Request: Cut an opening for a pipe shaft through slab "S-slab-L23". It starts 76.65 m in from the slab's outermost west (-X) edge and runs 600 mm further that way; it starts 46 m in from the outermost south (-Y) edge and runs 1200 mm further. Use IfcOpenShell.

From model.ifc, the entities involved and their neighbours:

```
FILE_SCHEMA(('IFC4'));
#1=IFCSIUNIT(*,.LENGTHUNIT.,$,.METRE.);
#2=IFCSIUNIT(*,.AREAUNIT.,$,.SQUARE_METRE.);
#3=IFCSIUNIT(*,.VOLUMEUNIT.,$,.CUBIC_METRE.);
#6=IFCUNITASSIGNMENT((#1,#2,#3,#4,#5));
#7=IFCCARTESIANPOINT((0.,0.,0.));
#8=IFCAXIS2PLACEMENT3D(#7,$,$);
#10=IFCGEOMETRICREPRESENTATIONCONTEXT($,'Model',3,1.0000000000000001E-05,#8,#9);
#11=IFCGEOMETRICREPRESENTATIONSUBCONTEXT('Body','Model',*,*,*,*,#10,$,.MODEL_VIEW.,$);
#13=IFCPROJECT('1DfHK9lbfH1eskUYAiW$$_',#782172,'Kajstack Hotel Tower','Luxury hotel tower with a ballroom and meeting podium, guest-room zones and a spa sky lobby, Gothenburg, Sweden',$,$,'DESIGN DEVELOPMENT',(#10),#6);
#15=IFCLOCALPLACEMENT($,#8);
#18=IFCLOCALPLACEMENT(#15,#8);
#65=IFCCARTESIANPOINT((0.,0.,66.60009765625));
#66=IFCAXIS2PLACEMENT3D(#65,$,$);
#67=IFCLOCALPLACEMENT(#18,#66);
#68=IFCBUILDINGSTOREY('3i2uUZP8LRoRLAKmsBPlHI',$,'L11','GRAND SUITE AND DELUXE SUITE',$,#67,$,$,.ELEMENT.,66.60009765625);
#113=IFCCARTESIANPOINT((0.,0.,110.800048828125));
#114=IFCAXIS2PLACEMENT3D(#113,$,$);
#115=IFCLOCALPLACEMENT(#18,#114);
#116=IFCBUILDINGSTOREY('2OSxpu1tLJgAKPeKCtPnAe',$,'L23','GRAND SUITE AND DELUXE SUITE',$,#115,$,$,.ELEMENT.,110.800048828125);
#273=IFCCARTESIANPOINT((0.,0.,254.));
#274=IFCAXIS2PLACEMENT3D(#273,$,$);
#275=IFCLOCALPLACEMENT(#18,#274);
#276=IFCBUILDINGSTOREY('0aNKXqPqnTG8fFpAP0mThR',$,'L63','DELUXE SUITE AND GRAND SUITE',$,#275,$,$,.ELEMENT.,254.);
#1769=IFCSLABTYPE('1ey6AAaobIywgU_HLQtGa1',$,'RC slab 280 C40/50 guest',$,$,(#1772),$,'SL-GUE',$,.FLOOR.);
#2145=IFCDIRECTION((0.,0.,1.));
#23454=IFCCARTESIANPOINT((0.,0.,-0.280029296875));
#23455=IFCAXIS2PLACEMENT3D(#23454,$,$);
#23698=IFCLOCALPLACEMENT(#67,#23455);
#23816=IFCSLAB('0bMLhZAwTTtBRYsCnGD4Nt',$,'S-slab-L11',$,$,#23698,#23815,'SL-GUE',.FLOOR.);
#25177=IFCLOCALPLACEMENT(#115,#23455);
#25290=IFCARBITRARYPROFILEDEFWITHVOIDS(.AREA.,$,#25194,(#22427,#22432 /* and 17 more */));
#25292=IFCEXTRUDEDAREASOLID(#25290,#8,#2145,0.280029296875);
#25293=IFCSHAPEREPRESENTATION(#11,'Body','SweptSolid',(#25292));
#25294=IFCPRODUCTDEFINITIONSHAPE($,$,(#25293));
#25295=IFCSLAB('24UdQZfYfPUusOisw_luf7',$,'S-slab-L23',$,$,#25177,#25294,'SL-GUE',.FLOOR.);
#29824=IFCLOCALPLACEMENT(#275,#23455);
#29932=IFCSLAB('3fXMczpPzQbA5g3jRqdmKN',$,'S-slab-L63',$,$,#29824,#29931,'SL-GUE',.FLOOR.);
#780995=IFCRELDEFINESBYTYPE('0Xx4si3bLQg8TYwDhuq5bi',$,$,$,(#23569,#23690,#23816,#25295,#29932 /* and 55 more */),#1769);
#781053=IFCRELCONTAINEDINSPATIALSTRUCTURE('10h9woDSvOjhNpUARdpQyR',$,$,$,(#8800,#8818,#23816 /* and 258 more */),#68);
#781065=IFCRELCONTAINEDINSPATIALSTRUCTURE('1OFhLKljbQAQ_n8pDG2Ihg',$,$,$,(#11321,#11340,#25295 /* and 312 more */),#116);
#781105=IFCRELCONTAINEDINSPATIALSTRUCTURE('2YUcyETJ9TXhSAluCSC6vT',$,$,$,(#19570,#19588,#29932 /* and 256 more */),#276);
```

```python
import numpy as np
import ifcopenshell
import ifcopenshell.api.feature
import ifcopenshell.api.geometry
import ifcopenshell.api.root
import ifcopenshell.geom
import ifcopenshell.util.placement
import ifcopenshell.util.representation
import ifcopenshell.util.shape
import ifcopenshell.util.unit

model = ifcopenshell.open("model.ifc")
unit_scale = ifcopenshell.util.unit.calculate_unit_scale(model)
settings = ifcopenshell.geom.settings()


def volume(element):
    """Net volume in cubic metres, openings subtracted."""
    shape = ifcopenshell.geom.create_shape(settings, element)
    return ifcopenshell.util.shape.get_volume(shape.geometry)


slab = model.by_id(25295)
before = volume(slab)

# Extent in the slab's own axes, in metres. The edges named are its -X and -Y sides.
slab_shape = ifcopenshell.geom.create_shape(settings, slab)
vertices = ifcopenshell.util.shape.get_vertices(slab_shape.geometry)
x_min, y_min, bottom = vertices.min(axis=0)
top = vertices[:, 2].max()

opening = ifcopenshell.api.root.create_entity(model, ifc_class="IfcOpeningElement", name="Pipe shaft opening", predefined_type="OPENING")
context = ifcopenshell.util.representation.get_context(model, "Model", "Body", "MODEL_VIEW")
width, depth = 0.6, 1.2
outline = [(0.0, 0.0), (width, 0.0), (width, depth), (0.0, depth), (0.0, 0.0)]
# Overshoot both faces by 50 mm so the cut is clean.
shape = ifcopenshell.api.geometry.add_slab_representation(
    model, context=context, depth=top - bottom + 0.1, polyline=outline
)
ifcopenshell.api.geometry.assign_representation(model, product=opening, representation=shape)

matrix = ifcopenshell.util.placement.get_local_placement(slab.ObjectPlacement)
matrix[:, 3] = matrix @ np.append(np.array([x_min + 76.65, y_min + 46, bottom - 0.05]) / unit_scale, 1.0)
ifcopenshell.api.geometry.edit_object_placement(model, product=opening, matrix=matrix, is_si=False)
ifcopenshell.api.feature.add_feature(model, feature=opening, element=slab)

after = volume(slab)

print(f"slab volume {before:.3f} -> {after:.3f} m3")

model.write("model-out.ifc")
```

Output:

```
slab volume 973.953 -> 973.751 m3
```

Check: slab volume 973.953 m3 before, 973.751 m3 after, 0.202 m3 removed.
